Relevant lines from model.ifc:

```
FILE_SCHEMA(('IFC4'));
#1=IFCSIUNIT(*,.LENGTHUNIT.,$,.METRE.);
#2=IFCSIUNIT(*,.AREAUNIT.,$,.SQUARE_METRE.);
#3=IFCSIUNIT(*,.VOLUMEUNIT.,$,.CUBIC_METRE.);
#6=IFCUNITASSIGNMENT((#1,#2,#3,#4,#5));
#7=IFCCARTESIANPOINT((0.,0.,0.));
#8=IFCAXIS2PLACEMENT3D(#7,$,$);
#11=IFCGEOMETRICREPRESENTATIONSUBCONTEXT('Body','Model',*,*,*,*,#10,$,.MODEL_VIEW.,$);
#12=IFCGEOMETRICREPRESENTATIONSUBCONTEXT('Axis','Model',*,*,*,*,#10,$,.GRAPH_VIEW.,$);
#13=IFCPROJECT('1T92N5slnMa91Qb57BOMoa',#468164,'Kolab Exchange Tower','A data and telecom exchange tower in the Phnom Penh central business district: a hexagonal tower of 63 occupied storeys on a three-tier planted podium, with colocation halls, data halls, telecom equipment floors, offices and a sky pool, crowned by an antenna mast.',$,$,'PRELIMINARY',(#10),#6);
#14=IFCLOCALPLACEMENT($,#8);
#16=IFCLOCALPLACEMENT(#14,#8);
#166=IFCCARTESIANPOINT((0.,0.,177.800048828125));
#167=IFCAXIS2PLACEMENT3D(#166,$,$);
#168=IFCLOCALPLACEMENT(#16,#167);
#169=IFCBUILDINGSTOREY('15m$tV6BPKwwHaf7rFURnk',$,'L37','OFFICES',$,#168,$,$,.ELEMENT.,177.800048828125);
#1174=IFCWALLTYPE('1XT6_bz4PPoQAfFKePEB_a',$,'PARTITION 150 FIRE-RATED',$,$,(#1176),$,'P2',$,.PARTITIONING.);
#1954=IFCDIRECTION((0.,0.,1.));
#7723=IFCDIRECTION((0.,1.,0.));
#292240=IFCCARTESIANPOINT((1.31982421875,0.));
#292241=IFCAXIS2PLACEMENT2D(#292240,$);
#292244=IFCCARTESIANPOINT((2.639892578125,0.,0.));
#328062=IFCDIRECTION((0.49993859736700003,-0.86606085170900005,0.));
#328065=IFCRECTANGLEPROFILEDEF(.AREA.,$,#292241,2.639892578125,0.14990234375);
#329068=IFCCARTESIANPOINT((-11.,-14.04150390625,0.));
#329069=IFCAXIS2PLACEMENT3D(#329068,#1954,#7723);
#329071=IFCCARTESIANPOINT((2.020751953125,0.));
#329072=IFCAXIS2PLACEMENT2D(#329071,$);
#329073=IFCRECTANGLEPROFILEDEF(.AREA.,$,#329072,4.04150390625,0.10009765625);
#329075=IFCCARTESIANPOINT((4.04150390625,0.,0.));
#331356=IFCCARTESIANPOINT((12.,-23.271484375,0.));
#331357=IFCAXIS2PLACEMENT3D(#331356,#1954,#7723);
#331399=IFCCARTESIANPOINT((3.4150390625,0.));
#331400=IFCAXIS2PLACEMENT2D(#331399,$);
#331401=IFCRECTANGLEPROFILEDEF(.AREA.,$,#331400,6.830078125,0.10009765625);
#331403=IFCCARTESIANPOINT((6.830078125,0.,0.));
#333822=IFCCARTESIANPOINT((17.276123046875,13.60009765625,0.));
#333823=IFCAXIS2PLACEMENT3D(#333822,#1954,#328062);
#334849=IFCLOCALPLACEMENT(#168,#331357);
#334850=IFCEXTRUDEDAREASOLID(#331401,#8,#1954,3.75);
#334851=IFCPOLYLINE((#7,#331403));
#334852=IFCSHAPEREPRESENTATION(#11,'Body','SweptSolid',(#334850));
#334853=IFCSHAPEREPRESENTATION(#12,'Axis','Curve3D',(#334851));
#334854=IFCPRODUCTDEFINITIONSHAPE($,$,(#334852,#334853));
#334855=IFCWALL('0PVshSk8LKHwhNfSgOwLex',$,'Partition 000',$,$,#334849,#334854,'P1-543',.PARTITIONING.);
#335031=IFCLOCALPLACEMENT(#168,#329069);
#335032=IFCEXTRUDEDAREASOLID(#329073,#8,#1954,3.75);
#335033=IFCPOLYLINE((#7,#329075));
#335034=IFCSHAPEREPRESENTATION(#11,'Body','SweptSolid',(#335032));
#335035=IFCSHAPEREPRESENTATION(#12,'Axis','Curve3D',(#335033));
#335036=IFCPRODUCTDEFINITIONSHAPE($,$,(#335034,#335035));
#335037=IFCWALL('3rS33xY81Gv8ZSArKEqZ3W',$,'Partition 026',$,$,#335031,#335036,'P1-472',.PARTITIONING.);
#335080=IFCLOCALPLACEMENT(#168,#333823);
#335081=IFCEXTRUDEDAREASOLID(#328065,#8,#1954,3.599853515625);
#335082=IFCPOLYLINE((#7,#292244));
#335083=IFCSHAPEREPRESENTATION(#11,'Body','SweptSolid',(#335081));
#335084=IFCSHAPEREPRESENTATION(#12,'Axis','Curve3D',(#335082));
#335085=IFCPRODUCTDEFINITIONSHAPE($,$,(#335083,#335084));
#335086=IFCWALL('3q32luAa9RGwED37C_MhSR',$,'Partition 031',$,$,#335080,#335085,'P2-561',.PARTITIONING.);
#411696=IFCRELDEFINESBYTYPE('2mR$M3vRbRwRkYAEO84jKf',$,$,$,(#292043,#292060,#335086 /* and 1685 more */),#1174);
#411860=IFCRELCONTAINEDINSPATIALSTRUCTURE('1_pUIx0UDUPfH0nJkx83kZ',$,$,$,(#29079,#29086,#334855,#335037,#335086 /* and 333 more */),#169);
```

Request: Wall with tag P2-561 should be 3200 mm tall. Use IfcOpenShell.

```python
import ifcopenshell
import ifcopenshell.geom
import ifcopenshell.util.representation
import ifcopenshell.util.shape
import ifcopenshell.util.unit

model = ifcopenshell.open("model.ifc")
unit_scale = ifcopenshell.util.unit.calculate_unit_scale(model)
settings = ifcopenshell.geom.settings()


def volume(element):
    """Net volume in cubic metres, openings subtracted."""
    shape = ifcopenshell.geom.create_shape(settings, element)
    return ifcopenshell.util.shape.get_volume(shape.geometry)


wall = model.by_guid("3q32luAa9RGwED37C_MhSR")
before = volume(wall)

body = ifcopenshell.util.representation.get_representation(wall, "Model", "Body")
solid = body.Items[0]
old_height = solid.Depth
solid.Depth = 3.2 / unit_scale
after = volume(wall)

print(f"height {old_height:g} -> {solid.Depth:g}, volume {before:.3f} -> {after:.3f} m3")

model.write("model_edited.ifc")
```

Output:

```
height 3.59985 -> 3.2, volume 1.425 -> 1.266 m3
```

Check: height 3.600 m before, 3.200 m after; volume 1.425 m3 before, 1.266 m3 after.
